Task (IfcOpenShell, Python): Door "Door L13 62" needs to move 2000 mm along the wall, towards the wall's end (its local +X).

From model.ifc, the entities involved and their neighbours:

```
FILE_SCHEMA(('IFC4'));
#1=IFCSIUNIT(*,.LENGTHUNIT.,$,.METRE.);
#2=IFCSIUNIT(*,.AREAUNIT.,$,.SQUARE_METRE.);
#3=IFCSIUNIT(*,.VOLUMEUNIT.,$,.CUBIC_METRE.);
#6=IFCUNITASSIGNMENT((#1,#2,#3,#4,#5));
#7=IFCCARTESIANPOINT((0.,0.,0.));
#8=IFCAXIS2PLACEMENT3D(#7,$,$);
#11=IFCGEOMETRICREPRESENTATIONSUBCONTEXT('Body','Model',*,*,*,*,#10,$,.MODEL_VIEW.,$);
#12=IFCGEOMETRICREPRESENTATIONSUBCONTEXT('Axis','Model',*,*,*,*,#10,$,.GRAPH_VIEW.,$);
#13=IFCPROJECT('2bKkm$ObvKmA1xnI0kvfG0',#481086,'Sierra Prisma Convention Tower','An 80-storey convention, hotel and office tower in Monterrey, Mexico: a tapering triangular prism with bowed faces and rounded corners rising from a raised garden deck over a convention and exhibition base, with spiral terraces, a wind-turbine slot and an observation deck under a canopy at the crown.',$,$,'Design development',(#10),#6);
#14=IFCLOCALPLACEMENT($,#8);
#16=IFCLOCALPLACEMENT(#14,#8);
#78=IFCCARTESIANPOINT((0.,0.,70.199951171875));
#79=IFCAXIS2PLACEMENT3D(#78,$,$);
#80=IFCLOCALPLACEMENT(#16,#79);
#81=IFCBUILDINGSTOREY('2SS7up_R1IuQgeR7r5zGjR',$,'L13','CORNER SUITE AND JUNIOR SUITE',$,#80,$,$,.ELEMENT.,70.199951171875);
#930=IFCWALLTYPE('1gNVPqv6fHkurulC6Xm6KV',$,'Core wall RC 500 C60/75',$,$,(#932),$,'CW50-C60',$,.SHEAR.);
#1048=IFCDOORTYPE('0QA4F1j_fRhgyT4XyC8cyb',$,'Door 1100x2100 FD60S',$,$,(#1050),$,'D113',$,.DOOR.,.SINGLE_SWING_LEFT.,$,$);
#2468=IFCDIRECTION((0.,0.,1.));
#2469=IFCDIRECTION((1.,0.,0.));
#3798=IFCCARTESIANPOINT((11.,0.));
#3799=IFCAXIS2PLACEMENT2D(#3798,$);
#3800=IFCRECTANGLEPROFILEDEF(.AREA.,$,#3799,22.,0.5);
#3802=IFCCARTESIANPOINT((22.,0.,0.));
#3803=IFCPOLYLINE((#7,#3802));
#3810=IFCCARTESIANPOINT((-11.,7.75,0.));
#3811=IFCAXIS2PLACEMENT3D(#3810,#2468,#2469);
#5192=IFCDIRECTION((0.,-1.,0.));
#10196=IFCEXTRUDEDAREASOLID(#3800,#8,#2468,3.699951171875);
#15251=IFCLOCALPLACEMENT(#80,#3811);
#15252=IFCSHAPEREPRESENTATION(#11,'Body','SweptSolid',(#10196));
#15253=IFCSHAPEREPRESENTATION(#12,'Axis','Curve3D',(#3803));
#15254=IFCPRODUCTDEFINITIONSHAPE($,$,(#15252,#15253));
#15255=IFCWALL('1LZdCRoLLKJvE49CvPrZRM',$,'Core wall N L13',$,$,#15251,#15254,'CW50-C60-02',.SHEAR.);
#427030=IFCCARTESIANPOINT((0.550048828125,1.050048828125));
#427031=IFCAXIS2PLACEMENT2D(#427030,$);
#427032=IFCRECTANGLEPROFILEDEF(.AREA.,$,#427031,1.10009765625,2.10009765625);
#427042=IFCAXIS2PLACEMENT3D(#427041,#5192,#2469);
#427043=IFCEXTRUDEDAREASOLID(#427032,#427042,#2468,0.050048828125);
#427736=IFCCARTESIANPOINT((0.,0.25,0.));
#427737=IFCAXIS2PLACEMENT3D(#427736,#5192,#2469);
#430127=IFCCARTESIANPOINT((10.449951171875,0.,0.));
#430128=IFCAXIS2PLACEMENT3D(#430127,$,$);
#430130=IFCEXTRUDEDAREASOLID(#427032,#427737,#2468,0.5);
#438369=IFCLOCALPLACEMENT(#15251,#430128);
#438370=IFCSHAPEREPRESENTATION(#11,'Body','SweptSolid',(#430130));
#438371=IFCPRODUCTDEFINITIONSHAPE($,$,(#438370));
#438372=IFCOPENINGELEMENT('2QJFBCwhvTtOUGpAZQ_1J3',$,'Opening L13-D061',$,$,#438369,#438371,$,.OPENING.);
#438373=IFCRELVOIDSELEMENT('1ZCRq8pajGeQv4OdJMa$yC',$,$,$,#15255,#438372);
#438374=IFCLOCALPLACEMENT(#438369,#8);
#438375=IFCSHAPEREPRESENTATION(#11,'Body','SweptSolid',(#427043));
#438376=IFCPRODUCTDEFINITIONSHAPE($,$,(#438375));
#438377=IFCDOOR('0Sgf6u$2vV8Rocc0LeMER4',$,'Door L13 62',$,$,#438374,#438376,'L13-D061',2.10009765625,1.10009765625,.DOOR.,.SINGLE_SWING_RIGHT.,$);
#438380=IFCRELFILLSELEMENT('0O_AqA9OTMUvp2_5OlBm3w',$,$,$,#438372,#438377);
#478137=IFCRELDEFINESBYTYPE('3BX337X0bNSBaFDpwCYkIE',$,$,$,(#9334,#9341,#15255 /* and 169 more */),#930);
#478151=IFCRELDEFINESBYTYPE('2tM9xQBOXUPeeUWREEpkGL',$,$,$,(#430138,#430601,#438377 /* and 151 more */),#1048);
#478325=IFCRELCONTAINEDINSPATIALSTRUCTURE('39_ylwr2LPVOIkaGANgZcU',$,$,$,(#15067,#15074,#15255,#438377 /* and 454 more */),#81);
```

```python
import ifcopenshell
import ifcopenshell.api.geometry
import ifcopenshell.util.placement
import ifcopenshell.util.unit

model = ifcopenshell.open("model.ifc")
unit_scale = ifcopenshell.util.unit.calculate_unit_scale(model)

door = model.by_id(438377)
opening = door.FillsVoids[0].RelatingOpeningElement
wall = opening.VoidsElements[0].RelatingBuildingElement

wall_matrix = ifcopenshell.util.placement.get_local_placement(wall.ObjectPlacement)
shift = wall_matrix[:3, 0] * 2 / unit_scale
before = ifcopenshell.util.placement.get_local_placement(door.ObjectPlacement)[:3, 3].copy()

# The door is placed relative to its opening, so it follows when the opening moves.
matrix = ifcopenshell.util.placement.get_local_placement(opening.ObjectPlacement)
matrix[:3, 3] += shift
ifcopenshell.api.geometry.edit_object_placement(
    model, product=opening, matrix=matrix, is_si=False, should_transform_children=True
)

after = ifcopenshell.util.placement.get_local_placement(door.ObjectPlacement)[:3, 3]
print("door moved by", (after - before).round(3) + 0.0)

model.write("model_edited.ifc")
```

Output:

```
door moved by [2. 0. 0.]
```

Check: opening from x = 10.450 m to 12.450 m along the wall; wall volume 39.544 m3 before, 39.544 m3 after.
